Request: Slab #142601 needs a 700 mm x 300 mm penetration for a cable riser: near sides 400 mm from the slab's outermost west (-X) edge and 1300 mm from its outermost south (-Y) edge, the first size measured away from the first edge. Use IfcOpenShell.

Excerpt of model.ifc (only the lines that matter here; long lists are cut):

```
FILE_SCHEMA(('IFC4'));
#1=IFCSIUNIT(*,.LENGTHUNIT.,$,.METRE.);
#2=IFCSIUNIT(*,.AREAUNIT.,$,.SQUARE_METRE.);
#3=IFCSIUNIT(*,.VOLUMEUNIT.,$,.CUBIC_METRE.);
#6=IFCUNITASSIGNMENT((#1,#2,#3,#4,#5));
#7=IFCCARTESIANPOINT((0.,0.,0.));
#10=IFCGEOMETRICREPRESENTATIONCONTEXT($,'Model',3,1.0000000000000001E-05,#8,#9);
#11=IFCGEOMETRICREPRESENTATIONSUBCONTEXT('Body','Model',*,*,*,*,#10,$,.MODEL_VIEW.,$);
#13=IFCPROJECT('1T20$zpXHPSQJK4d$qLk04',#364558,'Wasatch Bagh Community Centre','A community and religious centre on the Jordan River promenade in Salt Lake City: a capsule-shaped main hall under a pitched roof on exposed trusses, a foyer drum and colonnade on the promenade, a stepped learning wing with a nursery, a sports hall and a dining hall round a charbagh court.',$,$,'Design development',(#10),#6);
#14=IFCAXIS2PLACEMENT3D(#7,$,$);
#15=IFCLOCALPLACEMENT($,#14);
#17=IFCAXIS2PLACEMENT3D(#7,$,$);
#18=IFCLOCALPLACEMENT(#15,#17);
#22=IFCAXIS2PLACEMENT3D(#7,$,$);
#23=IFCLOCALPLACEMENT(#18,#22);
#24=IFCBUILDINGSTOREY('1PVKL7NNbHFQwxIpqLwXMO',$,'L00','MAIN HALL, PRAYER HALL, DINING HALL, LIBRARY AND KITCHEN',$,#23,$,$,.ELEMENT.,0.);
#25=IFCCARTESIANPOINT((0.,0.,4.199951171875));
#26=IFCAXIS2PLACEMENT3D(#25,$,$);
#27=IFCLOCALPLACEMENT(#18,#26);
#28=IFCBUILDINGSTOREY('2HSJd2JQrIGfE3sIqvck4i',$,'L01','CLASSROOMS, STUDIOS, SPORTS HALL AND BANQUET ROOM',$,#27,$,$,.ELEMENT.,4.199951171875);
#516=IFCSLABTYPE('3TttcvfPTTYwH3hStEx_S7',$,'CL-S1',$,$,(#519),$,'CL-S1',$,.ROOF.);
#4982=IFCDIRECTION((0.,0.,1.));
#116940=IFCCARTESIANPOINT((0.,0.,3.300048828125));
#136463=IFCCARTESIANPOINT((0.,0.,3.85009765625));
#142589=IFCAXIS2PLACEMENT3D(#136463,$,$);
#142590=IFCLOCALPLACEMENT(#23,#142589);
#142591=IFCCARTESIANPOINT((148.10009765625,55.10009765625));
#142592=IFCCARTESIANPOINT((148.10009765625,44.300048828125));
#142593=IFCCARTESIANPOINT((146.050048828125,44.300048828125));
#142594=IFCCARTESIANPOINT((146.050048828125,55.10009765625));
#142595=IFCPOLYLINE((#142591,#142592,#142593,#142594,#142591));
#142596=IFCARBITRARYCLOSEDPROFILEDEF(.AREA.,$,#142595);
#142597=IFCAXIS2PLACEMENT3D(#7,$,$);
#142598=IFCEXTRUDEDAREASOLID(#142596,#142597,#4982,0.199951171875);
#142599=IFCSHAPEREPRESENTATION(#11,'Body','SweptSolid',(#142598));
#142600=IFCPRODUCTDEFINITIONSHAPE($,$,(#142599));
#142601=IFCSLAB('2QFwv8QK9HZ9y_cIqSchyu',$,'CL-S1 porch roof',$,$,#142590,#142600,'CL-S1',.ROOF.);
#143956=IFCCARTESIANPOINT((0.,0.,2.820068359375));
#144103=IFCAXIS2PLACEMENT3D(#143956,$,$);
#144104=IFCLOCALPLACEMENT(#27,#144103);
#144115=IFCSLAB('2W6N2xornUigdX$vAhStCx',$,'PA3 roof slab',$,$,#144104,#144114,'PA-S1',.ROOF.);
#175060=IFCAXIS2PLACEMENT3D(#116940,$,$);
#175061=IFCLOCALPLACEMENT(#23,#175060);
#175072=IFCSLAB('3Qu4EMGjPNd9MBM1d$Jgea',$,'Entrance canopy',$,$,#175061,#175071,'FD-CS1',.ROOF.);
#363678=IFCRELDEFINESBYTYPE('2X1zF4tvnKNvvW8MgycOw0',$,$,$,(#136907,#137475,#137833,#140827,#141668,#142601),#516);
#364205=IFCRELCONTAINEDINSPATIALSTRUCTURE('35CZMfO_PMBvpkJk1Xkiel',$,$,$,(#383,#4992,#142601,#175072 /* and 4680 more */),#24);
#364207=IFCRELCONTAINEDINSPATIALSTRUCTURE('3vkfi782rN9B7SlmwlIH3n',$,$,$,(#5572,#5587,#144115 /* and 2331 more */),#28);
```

```python
import numpy as np
import ifcopenshell
import ifcopenshell.api.feature
import ifcopenshell.api.geometry
import ifcopenshell.api.root
import ifcopenshell.geom
import ifcopenshell.util.placement
import ifcopenshell.util.representation
import ifcopenshell.util.shape
import ifcopenshell.util.unit

model = ifcopenshell.open("model.ifc")
unit_scale = ifcopenshell.util.unit.calculate_unit_scale(model)
settings = ifcopenshell.geom.settings()


def volume(element):
    """Net volume in cubic metres, openings subtracted."""
    shape = ifcopenshell.geom.create_shape(settings, element)
    return ifcopenshell.util.shape.get_volume(shape.geometry)


slab = model.by_guid("2QFwv8QK9HZ9y_cIqSchyu")
before = volume(slab)

# Extent in the slab's own axes, in metres. The edges named are its -X and -Y sides.
slab_shape = ifcopenshell.geom.create_shape(settings, slab)
vertices = ifcopenshell.util.shape.get_vertices(slab_shape.geometry)
x_min, y_min, bottom = vertices.min(axis=0)
top = vertices[:, 2].max()

opening = ifcopenshell.api.root.create_entity(model, ifc_class="IfcOpeningElement", name="Cable riser opening", predefined_type="OPENING")
context = ifcopenshell.util.representation.get_context(model, "Model", "Body", "MODEL_VIEW")
width, depth = 0.7, 0.3
outline = [(0.0, 0.0), (width, 0.0), (width, depth), (0.0, depth), (0.0, 0.0)]
# Overshoot both faces by 50 mm so the cut is clean.
shape = ifcopenshell.api.geometry.add_slab_representation(
    model, context=context, depth=top - bottom + 0.1, polyline=outline
)
ifcopenshell.api.geometry.assign_representation(model, product=opening, representation=shape)

matrix = ifcopenshell.util.placement.get_local_placement(slab.ObjectPlacement)
matrix[:, 3] = matrix @ np.append(np.array([x_min + 0.4, y_min + 1.3, bottom - 0.05]) / unit_scale, 1.0)
ifcopenshell.api.geometry.edit_object_placement(model, product=opening, matrix=matrix, is_si=False)
ifcopenshell.api.feature.add_feature(model, feature=opening, element=slab)

after = volume(slab)

print(f"slab volume {before:.3f} -> {after:.3f} m3")

model.write("model-out.ifc")
```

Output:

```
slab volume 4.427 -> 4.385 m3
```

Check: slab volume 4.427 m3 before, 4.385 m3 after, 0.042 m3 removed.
